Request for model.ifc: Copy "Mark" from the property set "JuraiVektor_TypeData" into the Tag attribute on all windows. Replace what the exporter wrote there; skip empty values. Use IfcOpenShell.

First a look at what the model holds.

```python
import ifcopenshell
import ifcopenshell.util.element

model = ifcopenshell.open("model.ifc")
print(model.schema)
windows = model.by_type("IfcWindow")
print(len(windows), "windows")
for e in windows[:8]:
    source = ifcopenshell.util.element.get_pset(e, "JuraiVektor_TypeData", "Mark")
    target = e.Tag
    print(e.id(), repr(source), repr(target), sep=" | ")
```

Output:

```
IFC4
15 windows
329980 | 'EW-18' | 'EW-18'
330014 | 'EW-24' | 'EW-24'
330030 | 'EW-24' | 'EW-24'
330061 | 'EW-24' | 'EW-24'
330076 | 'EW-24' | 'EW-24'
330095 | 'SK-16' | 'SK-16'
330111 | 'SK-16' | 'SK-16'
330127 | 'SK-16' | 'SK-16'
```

```python
import ifcopenshell
import ifcopenshell.util.element

model = ifcopenshell.open("model.ifc")

count = 0
for e in model.by_type("IfcWindow"):
    value = ifcopenshell.util.element.get_pset(e, "JuraiVektor_TypeData", "Mark")
    current = e.Tag
    if not value or not value.strip() or current == value:
        continue
    e.Tag = value
    count += 1

print(count, "windows updated")

model.write("model_v2.ifc")
```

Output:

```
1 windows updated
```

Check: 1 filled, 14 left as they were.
